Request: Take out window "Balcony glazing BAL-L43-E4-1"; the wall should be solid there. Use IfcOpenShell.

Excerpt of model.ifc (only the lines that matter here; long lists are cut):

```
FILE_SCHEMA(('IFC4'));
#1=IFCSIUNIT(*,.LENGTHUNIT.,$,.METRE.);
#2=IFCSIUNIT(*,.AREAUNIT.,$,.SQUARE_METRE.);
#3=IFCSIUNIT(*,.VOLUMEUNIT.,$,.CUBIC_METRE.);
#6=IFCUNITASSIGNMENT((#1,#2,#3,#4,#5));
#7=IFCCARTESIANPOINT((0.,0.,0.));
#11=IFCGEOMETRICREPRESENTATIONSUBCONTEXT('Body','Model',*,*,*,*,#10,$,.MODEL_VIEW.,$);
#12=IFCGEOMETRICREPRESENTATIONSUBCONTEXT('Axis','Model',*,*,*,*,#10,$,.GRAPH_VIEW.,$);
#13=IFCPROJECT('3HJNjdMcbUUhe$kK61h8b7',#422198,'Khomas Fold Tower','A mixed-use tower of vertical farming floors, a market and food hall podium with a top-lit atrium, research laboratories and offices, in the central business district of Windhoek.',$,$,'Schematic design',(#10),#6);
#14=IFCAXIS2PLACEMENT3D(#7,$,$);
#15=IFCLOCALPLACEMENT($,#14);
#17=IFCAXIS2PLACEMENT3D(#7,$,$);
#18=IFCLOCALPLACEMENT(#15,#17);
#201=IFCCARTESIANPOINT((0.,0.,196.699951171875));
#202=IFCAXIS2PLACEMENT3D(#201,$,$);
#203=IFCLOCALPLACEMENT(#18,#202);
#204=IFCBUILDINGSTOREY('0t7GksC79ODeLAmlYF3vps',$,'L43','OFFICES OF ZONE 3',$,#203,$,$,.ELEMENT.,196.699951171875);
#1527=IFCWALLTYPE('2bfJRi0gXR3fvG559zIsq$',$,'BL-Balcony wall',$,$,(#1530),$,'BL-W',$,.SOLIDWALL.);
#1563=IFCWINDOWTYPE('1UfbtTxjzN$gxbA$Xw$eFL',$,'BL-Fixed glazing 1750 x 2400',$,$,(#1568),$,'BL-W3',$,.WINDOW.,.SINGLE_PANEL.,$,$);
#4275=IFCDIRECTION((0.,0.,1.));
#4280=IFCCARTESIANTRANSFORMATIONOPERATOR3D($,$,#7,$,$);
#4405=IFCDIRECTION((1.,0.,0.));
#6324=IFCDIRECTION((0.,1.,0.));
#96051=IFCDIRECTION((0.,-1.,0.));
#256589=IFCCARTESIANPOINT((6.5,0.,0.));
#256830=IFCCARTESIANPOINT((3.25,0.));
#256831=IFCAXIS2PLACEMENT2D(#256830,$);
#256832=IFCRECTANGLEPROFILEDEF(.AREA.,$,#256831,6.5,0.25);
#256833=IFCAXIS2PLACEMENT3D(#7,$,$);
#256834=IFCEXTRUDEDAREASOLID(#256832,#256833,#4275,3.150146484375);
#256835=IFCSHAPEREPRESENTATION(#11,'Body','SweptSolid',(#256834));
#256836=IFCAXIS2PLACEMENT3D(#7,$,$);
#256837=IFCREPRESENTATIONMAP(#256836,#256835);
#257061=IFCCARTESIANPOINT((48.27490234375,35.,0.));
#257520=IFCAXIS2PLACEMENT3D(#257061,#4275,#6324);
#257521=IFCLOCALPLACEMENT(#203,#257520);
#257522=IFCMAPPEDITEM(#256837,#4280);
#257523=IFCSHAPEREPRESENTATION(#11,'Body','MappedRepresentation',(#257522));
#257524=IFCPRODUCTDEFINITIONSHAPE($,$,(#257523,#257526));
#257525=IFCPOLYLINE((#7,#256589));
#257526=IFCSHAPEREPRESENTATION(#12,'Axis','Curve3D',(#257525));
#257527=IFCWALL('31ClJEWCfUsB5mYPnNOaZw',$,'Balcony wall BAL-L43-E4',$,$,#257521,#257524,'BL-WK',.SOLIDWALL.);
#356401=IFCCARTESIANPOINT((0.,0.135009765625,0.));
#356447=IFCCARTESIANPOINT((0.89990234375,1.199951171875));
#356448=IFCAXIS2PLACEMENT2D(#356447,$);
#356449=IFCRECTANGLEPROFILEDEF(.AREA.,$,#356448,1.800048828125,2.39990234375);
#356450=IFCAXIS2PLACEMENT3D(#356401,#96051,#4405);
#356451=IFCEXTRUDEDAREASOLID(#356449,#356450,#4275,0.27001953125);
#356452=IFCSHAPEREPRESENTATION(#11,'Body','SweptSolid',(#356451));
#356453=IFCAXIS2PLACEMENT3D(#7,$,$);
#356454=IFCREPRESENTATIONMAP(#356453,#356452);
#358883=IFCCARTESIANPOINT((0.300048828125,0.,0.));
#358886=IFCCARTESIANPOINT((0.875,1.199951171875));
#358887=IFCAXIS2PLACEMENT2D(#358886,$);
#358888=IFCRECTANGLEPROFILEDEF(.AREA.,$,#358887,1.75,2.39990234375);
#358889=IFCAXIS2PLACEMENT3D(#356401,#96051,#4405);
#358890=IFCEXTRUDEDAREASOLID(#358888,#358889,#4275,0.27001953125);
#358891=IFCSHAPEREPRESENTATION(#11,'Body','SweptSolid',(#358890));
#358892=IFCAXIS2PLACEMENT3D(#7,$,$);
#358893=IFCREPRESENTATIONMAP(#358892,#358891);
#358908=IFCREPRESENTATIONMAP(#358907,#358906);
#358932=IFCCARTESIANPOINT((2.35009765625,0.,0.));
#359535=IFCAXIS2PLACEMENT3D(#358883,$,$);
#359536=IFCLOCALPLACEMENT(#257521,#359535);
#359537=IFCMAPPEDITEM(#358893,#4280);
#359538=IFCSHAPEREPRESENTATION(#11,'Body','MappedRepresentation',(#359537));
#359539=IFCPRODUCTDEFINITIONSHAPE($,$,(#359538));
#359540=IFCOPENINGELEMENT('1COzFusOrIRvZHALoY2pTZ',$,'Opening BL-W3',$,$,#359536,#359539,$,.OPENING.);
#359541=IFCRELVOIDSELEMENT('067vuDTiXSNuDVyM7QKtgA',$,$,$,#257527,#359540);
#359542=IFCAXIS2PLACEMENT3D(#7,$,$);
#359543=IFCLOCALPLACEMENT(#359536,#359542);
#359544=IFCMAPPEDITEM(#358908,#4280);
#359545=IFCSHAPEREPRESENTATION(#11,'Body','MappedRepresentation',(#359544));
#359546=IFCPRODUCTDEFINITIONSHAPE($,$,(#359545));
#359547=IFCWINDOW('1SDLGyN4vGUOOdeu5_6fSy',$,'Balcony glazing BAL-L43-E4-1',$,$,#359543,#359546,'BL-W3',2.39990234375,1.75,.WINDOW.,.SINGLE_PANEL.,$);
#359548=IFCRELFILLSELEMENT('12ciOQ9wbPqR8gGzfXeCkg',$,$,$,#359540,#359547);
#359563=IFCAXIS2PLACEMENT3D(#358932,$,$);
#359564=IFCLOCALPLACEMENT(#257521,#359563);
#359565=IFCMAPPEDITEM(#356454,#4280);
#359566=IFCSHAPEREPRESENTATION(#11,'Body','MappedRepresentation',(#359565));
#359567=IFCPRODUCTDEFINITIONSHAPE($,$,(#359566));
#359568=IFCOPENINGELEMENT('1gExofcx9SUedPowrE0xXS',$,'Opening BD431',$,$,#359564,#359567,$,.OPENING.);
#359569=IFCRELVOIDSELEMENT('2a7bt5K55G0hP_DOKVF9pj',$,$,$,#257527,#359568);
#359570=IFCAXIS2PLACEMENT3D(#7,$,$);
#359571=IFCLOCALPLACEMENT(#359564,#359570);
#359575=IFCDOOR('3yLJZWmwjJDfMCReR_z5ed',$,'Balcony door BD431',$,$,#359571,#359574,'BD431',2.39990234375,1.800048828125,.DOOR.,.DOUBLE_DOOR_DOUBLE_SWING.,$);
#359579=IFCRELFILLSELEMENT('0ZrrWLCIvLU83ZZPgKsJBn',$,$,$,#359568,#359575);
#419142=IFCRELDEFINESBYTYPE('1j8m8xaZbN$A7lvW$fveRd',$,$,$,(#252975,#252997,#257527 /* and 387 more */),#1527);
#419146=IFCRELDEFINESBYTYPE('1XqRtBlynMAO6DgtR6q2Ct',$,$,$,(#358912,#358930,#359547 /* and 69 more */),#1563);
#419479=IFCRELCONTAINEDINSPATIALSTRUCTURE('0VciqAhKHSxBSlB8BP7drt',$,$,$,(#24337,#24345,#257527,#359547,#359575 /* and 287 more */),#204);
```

```python
import ifcopenshell
import ifcopenshell.api.feature
import ifcopenshell.api.root
import ifcopenshell.geom
import ifcopenshell.util.shape

model = ifcopenshell.open("model.ifc")
settings = ifcopenshell.geom.settings()


def volume(element):
    """Net volume in cubic metres, openings subtracted."""
    shape = ifcopenshell.geom.create_shape(settings, element)
    return ifcopenshell.util.shape.get_volume(shape.geometry)


window = model.by_guid("1SDLGyN4vGUOOdeu5_6fSy")
opening = window.FillsVoids[0].RelatingOpeningElement
wall = opening.VoidsElements[0].RelatingBuildingElement
before = volume(wall)

ifcopenshell.api.root.remove_product(model, product=window)
ifcopenshell.api.feature.remove_feature(model, feature=opening)

after = volume(wall)

print(f"wall volume {before:.3f} -> {after:.3f} m3")

model.write("model-out.ifc")
```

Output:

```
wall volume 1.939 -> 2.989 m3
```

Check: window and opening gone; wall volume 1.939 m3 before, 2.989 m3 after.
